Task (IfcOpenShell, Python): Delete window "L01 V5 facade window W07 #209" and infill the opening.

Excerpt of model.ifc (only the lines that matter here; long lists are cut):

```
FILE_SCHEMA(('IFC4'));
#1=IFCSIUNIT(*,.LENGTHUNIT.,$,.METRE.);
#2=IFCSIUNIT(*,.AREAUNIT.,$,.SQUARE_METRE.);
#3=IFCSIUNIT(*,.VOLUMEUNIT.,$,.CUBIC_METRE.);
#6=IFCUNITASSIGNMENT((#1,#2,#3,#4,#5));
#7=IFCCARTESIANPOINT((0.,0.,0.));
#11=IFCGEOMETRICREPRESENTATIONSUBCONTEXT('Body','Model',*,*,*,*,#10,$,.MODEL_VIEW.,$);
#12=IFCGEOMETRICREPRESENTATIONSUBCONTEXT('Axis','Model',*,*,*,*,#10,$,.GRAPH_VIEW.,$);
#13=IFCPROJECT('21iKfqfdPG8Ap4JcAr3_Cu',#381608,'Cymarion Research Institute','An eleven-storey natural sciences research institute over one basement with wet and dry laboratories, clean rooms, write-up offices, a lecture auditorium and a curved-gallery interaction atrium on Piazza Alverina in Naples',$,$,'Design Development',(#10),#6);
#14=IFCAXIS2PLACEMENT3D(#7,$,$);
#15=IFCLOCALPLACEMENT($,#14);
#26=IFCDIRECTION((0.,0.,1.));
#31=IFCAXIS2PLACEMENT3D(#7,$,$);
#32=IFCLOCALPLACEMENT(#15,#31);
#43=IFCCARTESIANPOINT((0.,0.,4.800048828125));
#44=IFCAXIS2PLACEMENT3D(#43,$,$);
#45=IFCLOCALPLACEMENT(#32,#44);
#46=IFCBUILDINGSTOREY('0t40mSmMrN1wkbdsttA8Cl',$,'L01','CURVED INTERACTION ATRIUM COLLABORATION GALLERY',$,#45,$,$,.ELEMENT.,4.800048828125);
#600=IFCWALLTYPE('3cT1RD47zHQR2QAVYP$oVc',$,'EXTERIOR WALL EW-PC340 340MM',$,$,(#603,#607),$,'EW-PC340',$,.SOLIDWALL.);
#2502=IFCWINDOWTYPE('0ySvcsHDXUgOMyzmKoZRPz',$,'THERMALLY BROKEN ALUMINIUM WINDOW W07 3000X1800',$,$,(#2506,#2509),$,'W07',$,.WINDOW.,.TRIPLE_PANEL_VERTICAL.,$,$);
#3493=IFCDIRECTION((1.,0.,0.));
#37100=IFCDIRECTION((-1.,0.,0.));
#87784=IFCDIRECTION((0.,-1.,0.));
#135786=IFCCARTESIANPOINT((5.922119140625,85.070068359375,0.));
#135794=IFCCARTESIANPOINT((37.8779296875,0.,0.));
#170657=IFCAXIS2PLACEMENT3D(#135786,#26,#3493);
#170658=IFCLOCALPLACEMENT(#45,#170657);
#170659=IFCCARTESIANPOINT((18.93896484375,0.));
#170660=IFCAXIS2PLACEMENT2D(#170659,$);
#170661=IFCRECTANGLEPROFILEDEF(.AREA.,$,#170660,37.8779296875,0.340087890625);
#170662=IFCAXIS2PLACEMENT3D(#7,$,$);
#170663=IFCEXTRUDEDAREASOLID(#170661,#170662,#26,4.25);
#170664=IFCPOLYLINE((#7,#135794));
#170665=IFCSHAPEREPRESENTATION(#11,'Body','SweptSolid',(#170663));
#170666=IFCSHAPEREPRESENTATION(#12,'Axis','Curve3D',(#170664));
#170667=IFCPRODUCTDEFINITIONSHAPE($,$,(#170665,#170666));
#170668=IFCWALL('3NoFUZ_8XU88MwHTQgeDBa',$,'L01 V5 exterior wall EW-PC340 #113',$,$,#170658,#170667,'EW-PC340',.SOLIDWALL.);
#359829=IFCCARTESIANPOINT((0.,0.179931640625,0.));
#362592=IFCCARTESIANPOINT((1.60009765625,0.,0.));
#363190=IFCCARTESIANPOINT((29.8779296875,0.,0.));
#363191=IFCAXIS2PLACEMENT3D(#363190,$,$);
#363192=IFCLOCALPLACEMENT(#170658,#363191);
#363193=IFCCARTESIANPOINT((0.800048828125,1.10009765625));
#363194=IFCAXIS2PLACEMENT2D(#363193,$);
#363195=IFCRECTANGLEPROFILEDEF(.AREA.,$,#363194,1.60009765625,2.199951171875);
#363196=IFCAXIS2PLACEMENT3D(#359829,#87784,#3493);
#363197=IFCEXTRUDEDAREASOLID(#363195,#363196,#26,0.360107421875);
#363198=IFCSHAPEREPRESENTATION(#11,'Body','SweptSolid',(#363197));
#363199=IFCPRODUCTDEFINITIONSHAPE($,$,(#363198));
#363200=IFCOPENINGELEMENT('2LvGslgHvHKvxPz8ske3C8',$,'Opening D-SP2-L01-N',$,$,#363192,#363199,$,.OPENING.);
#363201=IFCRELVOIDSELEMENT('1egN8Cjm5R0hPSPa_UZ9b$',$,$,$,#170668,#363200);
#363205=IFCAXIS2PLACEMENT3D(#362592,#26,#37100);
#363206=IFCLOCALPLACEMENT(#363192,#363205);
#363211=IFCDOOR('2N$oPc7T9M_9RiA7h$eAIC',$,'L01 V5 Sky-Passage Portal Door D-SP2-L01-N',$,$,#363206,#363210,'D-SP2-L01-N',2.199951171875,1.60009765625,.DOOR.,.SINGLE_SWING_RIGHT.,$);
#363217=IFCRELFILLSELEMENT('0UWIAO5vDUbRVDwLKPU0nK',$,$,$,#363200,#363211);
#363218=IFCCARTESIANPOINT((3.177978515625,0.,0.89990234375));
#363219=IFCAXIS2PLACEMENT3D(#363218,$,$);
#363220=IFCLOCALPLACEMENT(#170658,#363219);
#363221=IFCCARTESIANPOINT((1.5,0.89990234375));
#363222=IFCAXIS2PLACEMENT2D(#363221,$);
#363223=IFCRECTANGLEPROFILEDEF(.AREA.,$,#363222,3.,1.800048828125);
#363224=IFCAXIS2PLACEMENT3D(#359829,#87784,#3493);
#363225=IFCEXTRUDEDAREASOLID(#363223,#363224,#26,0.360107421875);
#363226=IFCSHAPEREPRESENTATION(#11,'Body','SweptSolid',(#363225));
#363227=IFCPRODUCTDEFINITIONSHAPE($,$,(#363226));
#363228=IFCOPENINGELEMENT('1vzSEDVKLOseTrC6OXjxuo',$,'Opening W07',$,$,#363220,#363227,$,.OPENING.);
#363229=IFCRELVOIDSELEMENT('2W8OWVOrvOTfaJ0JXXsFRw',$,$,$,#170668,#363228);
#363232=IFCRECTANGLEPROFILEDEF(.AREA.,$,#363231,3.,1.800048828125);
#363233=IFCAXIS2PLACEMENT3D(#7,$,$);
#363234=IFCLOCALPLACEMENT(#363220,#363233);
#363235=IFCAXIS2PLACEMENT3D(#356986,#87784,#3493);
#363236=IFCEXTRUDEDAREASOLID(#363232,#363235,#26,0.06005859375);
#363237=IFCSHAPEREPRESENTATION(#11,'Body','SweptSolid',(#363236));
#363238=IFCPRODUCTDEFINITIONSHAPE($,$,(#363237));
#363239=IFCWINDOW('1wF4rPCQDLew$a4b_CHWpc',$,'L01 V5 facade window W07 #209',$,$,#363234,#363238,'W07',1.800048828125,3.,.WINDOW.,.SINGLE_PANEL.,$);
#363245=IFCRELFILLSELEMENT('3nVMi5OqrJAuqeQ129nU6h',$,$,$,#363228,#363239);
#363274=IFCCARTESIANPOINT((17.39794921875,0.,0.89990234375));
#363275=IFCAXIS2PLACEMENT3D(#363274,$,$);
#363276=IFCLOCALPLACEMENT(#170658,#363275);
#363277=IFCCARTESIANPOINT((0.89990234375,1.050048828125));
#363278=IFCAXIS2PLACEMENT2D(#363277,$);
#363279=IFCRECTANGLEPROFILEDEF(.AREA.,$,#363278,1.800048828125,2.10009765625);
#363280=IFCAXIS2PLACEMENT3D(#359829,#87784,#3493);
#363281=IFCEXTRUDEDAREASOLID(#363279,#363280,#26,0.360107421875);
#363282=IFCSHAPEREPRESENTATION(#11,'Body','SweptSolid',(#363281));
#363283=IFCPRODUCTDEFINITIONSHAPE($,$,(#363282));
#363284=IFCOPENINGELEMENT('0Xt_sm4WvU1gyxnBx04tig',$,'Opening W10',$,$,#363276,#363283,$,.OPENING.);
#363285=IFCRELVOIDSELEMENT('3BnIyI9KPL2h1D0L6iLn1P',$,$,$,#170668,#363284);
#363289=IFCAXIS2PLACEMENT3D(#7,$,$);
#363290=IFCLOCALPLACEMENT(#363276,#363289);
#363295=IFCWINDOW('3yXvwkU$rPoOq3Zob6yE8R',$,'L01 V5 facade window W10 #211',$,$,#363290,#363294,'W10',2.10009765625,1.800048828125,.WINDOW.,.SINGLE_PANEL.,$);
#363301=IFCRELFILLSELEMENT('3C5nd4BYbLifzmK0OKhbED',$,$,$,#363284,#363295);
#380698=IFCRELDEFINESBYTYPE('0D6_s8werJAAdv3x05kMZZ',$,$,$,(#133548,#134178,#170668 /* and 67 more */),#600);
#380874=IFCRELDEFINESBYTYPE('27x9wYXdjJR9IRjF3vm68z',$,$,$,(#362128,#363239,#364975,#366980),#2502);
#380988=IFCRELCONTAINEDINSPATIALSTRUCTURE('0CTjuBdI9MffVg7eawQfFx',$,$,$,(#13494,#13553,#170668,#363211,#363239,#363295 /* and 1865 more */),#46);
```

```python
import ifcopenshell
import ifcopenshell.api.feature
import ifcopenshell.api.root
import ifcopenshell.geom
import ifcopenshell.util.shape

model = ifcopenshell.open("model.ifc")
settings = ifcopenshell.geom.settings()


def volume(element):
    """Net volume in cubic metres, openings subtracted."""
    shape = ifcopenshell.geom.create_shape(settings, element)
    return ifcopenshell.util.shape.get_volume(shape.geometry)


window = model.by_guid("1wF4rPCQDLew$a4b_CHWpc")
opening = window.FillsVoids[0].RelatingOpeningElement
wall = opening.VoidsElements[0].RelatingBuildingElement
before = volume(wall)

ifcopenshell.api.root.remove_product(model, product=window)
ifcopenshell.api.feature.remove_feature(model, feature=opening)

after = volume(wall)

print(f"wall volume {before:.3f} -> {after:.3f} m3")

model.write("model_v2.ifc")
```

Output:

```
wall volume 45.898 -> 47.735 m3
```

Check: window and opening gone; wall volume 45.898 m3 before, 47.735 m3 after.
